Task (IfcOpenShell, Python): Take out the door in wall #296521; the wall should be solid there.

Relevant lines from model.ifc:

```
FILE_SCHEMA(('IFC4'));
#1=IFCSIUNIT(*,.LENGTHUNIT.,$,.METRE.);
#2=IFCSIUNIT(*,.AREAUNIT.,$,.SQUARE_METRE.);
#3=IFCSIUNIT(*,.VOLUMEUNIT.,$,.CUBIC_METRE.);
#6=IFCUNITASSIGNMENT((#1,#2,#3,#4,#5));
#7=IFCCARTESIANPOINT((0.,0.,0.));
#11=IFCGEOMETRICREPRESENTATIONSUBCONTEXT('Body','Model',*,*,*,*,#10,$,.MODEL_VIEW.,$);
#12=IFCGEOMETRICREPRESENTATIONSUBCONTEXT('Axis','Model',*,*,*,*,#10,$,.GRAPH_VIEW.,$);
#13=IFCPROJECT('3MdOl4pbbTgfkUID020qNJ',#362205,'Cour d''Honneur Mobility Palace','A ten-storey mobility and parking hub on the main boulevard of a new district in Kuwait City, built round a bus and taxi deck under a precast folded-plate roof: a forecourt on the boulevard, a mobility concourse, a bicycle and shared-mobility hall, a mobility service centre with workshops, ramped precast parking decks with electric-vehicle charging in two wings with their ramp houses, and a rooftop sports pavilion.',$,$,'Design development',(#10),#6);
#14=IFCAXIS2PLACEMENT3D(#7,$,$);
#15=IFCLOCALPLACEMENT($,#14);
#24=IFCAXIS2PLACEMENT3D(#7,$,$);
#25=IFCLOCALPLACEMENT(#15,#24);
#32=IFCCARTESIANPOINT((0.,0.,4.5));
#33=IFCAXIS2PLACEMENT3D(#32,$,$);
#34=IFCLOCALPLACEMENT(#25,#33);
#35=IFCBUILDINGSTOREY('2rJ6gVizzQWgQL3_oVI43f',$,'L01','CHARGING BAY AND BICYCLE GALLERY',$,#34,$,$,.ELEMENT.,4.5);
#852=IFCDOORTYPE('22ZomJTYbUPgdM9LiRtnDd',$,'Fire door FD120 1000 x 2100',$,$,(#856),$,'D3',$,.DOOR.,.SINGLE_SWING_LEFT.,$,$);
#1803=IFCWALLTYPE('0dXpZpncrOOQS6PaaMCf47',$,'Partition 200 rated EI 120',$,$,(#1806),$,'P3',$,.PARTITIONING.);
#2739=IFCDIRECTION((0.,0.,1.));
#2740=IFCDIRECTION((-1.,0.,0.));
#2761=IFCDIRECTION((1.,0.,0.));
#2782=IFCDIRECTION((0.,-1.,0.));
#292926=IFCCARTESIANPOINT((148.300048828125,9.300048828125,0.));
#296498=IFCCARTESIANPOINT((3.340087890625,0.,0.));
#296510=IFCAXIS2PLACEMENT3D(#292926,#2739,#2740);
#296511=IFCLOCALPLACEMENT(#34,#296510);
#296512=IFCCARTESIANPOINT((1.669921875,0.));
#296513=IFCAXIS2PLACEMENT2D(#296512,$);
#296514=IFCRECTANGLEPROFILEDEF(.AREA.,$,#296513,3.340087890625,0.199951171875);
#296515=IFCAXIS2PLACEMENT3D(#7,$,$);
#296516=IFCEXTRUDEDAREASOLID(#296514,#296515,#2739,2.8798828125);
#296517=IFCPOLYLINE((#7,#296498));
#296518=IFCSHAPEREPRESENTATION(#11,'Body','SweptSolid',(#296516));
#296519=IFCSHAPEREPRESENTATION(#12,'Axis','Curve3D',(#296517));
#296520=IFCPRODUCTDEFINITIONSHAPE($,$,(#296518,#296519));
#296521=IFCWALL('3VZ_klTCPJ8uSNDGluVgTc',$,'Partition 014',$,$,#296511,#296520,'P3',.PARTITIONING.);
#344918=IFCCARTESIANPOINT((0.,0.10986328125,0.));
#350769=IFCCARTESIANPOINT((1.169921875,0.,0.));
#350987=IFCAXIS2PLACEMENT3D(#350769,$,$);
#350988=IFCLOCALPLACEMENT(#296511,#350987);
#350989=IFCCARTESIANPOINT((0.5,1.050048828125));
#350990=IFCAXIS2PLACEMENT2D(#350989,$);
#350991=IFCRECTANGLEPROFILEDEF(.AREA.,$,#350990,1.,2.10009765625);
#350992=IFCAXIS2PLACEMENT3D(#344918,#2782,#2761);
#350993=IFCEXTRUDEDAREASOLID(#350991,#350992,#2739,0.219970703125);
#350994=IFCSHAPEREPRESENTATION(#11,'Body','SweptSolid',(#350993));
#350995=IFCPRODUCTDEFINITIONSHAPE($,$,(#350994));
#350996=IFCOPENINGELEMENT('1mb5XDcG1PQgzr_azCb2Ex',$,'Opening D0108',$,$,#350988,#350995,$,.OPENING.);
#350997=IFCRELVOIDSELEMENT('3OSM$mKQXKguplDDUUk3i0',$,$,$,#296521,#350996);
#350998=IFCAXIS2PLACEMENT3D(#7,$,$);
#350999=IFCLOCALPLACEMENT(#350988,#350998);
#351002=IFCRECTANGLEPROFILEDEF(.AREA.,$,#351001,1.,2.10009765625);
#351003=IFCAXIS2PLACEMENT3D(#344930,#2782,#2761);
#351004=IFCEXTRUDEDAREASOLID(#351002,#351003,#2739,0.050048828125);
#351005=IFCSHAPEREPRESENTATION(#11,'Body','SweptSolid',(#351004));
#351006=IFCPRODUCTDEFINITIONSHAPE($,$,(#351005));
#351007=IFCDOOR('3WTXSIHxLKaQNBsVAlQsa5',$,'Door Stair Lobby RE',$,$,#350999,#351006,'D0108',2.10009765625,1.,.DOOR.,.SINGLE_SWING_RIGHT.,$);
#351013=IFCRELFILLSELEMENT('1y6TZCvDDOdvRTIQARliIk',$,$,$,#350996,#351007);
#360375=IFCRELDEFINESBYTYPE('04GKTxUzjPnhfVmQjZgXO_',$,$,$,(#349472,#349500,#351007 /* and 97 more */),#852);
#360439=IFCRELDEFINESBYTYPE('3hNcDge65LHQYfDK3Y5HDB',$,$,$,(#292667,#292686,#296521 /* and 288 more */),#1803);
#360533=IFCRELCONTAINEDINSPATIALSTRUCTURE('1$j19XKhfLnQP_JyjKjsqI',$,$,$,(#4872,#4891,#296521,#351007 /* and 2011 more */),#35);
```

```python
import ifcopenshell
import ifcopenshell.api.feature
import ifcopenshell.api.root
import ifcopenshell.geom
import ifcopenshell.util.shape

model = ifcopenshell.open("model.ifc")
settings = ifcopenshell.geom.settings()


def volume(element):
    """Net volume in cubic metres, openings subtracted."""
    shape = ifcopenshell.geom.create_shape(settings, element)
    return ifcopenshell.util.shape.get_volume(shape.geometry)


door = model.by_guid("3WTXSIHxLKaQNBsVAlQsa5")
opening = door.FillsVoids[0].RelatingOpeningElement
wall = opening.VoidsElements[0].RelatingBuildingElement
before = volume(wall)

ifcopenshell.api.root.remove_product(model, product=door)
ifcopenshell.api.feature.remove_feature(model, feature=opening)

after = volume(wall)

print(f"wall volume {before:.3f} -> {after:.3f} m3")

model.write("model-out.ifc")
```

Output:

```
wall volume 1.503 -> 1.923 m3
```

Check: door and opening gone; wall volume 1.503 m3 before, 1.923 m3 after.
